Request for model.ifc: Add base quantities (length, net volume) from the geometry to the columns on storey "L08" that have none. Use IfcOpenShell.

First a look at what the model holds.

```python
import ifcopenshell
import ifcopenshell.util.element
import ifcopenshell.util.unit

model = ifcopenshell.open("model.ifc")
print(model.schema)
for unit_type in ("LENGTHUNIT", "AREAUNIT", "VOLUMEUNIT"):
    print(unit_type, ifcopenshell.util.unit.calculate_unit_scale(model, unit_type))
storey = next(s for s in model.by_type("IfcBuildingStorey") if s.Name == "L08")
columns = [e for e in ifcopenshell.util.element.get_decomposition(storey) if e.is_a("IfcColumn")]
for e in sorted(columns, key=lambda e: e.id()):
    print(e.id(), e.is_a(), e.Name, list(ifcopenshell.util.element.get_psets(e, qtos_only=True)), sep=" | ")
```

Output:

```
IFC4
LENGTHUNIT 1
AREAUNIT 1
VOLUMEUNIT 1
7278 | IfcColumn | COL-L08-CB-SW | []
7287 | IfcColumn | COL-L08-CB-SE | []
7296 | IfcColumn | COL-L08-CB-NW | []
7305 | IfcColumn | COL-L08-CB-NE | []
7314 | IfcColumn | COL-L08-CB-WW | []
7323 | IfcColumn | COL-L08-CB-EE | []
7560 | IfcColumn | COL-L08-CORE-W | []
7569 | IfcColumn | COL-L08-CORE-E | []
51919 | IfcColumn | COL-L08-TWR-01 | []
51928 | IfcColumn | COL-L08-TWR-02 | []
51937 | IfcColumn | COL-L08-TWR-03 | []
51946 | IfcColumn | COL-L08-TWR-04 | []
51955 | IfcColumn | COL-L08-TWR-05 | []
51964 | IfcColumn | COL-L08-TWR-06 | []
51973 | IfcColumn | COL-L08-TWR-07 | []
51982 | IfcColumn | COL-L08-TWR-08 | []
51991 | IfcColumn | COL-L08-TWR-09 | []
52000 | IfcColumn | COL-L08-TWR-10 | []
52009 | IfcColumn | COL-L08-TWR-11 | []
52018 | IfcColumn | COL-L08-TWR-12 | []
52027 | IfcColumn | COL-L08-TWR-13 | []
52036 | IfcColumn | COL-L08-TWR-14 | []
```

```python
import ifcopenshell
import ifcopenshell.api.pset
import ifcopenshell.geom
import ifcopenshell.util.element
import ifcopenshell.util.shape
import ifcopenshell.util.unit

model = ifcopenshell.open("model.ifc")
unit_scale = ifcopenshell.util.unit.calculate_unit_scale(model)
volume_scale = ifcopenshell.util.unit.calculate_unit_scale(model, "VOLUMEUNIT")
settings = ifcopenshell.geom.settings()

storey = next(s for s in model.by_type("IfcBuildingStorey") if s.Name == "L08")
columns = [e for e in ifcopenshell.util.element.get_decomposition(storey) if e.is_a("IfcColumn")]

for e in sorted(columns, key=lambda e: e.id()):
    if ifcopenshell.util.element.get_psets(e, qtos_only=True, should_inherit=False):
        continue
    # Geometry comes back in metres, in the element's own axes.
    shape = ifcopenshell.geom.create_shape(settings, e)
    values = {
        "Length": ifcopenshell.util.shape.get_z(shape.geometry) / unit_scale,
        "NetVolume": ifcopenshell.util.shape.get_volume(shape.geometry) / volume_scale,
    }
    qto = ifcopenshell.api.pset.add_qto(model, product=e, name="Qto_ColumnBaseQuantities")
    ifcopenshell.api.pset.edit_qto(model, qto=qto, properties=values)
    print(e.id(), {k: round(v, 3) for k, v in values.items()})

model.write("model_rev.ifc")
```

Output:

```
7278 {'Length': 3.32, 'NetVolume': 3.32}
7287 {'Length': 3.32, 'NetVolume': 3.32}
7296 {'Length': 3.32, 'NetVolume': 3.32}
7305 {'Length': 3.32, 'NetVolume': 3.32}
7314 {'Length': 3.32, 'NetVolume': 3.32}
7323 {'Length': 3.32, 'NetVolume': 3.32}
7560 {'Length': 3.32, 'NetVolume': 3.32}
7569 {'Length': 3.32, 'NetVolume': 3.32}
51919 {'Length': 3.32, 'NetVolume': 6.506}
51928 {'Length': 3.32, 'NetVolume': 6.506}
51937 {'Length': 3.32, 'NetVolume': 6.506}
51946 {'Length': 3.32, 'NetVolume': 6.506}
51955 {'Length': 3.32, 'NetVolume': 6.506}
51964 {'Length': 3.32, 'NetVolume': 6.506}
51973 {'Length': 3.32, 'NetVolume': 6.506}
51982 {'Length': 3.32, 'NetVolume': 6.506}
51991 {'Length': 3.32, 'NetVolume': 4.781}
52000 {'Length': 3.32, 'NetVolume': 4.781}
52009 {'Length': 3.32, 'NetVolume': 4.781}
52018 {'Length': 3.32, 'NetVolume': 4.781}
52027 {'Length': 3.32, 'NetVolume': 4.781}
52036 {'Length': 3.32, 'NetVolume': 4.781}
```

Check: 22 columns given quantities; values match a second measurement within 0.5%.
